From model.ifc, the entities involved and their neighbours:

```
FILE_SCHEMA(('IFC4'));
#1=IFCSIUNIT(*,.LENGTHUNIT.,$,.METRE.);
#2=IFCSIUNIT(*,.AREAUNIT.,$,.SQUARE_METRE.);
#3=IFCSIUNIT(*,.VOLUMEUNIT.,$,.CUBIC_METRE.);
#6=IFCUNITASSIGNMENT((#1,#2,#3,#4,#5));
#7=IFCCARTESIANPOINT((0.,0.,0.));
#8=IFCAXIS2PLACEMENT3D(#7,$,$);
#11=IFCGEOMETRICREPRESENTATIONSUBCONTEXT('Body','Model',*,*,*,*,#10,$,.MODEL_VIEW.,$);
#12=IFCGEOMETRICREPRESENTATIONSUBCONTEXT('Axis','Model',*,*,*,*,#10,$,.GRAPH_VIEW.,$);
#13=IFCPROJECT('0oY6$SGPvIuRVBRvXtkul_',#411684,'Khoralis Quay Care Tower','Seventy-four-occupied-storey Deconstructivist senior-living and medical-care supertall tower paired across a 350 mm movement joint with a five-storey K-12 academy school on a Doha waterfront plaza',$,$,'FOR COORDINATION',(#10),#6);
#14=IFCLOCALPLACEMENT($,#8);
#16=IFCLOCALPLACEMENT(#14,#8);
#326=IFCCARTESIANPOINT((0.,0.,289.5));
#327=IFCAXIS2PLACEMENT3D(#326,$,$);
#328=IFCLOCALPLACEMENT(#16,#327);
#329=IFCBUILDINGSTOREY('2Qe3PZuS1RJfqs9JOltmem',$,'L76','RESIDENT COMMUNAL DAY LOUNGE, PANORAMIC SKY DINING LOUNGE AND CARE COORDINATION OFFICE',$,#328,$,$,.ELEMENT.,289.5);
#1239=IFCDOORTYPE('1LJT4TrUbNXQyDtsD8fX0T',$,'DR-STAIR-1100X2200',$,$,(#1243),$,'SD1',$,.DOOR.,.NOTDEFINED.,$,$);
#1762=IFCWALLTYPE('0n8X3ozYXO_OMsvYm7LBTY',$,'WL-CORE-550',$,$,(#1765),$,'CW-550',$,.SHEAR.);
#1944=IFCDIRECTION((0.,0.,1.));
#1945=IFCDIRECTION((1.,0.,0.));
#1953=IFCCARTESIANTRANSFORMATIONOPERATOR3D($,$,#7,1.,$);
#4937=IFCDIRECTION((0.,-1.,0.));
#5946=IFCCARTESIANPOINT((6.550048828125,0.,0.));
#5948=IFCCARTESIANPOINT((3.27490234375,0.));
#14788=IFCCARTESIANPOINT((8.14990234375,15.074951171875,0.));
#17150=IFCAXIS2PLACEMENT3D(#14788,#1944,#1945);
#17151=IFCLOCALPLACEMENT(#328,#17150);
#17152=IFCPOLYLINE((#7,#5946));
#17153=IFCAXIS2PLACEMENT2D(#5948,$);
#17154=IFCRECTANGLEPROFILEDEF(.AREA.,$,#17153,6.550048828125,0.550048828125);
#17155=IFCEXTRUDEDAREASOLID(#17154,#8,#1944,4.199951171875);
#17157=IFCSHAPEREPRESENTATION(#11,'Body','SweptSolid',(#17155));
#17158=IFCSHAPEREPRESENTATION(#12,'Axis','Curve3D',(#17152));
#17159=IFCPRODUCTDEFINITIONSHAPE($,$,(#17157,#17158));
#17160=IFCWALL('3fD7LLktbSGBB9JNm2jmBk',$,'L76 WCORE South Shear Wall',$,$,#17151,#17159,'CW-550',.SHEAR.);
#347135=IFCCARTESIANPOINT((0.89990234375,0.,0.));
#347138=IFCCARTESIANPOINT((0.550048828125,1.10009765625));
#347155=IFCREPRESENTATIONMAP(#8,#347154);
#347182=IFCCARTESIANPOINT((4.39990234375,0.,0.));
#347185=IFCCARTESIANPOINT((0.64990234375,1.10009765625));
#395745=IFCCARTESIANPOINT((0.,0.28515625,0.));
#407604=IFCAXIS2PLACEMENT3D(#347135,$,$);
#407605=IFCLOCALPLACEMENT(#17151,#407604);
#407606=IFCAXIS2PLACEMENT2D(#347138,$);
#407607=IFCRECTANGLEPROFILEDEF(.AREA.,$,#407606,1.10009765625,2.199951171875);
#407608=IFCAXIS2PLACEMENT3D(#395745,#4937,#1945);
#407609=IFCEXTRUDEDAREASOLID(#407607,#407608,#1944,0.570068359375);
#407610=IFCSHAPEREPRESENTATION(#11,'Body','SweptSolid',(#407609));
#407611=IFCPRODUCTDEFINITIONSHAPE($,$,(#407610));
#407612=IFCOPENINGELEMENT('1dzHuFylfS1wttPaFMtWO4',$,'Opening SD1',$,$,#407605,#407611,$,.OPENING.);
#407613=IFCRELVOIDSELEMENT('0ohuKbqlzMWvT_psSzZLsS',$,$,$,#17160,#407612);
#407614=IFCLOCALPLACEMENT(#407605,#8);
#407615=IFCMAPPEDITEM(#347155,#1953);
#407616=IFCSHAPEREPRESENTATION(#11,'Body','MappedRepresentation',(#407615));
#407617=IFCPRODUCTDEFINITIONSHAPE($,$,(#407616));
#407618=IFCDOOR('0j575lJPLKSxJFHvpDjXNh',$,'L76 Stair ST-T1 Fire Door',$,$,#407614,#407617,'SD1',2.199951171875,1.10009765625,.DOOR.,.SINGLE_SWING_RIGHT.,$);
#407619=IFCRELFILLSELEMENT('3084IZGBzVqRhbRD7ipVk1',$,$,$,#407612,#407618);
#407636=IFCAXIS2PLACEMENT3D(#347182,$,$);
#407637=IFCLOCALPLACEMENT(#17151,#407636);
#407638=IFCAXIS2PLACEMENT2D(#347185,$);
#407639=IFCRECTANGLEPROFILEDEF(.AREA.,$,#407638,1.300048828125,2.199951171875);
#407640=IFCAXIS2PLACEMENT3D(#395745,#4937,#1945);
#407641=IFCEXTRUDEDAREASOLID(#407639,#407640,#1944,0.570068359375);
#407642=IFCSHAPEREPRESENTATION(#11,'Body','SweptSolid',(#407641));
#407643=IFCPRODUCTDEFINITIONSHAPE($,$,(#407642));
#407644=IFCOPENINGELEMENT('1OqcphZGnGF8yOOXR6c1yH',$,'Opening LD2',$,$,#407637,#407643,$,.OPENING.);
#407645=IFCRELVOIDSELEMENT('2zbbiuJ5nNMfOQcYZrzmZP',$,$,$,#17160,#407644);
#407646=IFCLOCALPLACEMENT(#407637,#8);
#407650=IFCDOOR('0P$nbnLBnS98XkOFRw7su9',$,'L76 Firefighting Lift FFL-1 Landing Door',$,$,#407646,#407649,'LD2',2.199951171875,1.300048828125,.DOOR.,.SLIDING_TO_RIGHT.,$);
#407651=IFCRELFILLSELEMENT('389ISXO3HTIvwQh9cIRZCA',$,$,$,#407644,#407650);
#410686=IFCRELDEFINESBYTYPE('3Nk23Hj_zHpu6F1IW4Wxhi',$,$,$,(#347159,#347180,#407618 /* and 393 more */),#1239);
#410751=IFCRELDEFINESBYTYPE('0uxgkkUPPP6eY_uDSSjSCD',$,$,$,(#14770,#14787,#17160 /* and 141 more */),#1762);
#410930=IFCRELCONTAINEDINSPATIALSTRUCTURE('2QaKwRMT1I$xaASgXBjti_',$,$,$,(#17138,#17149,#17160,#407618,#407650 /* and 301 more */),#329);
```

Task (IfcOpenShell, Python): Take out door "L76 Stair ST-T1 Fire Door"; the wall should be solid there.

```python
import ifcopenshell
import ifcopenshell.api.feature
import ifcopenshell.api.root
import ifcopenshell.geom
import ifcopenshell.util.shape

model = ifcopenshell.open("model.ifc")
settings = ifcopenshell.geom.settings()


def volume(element):
    """Net volume in cubic metres, openings subtracted."""
    shape = ifcopenshell.geom.create_shape(settings, element)
    return ifcopenshell.util.shape.get_volume(shape.geometry)


door = model.by_guid("0j575lJPLKSxJFHvpDjXNh")
opening = door.FillsVoids[0].RelatingOpeningElement
wall = opening.VoidsElements[0].RelatingBuildingElement
before = volume(wall)

ifcopenshell.api.root.remove_product(model, product=door)
ifcopenshell.api.feature.remove_feature(model, feature=opening)

after = volume(wall)

print(f"wall volume {before:.3f} -> {after:.3f} m3")

model.write("model_v2.ifc")
```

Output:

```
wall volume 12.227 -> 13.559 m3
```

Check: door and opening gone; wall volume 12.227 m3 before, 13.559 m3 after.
